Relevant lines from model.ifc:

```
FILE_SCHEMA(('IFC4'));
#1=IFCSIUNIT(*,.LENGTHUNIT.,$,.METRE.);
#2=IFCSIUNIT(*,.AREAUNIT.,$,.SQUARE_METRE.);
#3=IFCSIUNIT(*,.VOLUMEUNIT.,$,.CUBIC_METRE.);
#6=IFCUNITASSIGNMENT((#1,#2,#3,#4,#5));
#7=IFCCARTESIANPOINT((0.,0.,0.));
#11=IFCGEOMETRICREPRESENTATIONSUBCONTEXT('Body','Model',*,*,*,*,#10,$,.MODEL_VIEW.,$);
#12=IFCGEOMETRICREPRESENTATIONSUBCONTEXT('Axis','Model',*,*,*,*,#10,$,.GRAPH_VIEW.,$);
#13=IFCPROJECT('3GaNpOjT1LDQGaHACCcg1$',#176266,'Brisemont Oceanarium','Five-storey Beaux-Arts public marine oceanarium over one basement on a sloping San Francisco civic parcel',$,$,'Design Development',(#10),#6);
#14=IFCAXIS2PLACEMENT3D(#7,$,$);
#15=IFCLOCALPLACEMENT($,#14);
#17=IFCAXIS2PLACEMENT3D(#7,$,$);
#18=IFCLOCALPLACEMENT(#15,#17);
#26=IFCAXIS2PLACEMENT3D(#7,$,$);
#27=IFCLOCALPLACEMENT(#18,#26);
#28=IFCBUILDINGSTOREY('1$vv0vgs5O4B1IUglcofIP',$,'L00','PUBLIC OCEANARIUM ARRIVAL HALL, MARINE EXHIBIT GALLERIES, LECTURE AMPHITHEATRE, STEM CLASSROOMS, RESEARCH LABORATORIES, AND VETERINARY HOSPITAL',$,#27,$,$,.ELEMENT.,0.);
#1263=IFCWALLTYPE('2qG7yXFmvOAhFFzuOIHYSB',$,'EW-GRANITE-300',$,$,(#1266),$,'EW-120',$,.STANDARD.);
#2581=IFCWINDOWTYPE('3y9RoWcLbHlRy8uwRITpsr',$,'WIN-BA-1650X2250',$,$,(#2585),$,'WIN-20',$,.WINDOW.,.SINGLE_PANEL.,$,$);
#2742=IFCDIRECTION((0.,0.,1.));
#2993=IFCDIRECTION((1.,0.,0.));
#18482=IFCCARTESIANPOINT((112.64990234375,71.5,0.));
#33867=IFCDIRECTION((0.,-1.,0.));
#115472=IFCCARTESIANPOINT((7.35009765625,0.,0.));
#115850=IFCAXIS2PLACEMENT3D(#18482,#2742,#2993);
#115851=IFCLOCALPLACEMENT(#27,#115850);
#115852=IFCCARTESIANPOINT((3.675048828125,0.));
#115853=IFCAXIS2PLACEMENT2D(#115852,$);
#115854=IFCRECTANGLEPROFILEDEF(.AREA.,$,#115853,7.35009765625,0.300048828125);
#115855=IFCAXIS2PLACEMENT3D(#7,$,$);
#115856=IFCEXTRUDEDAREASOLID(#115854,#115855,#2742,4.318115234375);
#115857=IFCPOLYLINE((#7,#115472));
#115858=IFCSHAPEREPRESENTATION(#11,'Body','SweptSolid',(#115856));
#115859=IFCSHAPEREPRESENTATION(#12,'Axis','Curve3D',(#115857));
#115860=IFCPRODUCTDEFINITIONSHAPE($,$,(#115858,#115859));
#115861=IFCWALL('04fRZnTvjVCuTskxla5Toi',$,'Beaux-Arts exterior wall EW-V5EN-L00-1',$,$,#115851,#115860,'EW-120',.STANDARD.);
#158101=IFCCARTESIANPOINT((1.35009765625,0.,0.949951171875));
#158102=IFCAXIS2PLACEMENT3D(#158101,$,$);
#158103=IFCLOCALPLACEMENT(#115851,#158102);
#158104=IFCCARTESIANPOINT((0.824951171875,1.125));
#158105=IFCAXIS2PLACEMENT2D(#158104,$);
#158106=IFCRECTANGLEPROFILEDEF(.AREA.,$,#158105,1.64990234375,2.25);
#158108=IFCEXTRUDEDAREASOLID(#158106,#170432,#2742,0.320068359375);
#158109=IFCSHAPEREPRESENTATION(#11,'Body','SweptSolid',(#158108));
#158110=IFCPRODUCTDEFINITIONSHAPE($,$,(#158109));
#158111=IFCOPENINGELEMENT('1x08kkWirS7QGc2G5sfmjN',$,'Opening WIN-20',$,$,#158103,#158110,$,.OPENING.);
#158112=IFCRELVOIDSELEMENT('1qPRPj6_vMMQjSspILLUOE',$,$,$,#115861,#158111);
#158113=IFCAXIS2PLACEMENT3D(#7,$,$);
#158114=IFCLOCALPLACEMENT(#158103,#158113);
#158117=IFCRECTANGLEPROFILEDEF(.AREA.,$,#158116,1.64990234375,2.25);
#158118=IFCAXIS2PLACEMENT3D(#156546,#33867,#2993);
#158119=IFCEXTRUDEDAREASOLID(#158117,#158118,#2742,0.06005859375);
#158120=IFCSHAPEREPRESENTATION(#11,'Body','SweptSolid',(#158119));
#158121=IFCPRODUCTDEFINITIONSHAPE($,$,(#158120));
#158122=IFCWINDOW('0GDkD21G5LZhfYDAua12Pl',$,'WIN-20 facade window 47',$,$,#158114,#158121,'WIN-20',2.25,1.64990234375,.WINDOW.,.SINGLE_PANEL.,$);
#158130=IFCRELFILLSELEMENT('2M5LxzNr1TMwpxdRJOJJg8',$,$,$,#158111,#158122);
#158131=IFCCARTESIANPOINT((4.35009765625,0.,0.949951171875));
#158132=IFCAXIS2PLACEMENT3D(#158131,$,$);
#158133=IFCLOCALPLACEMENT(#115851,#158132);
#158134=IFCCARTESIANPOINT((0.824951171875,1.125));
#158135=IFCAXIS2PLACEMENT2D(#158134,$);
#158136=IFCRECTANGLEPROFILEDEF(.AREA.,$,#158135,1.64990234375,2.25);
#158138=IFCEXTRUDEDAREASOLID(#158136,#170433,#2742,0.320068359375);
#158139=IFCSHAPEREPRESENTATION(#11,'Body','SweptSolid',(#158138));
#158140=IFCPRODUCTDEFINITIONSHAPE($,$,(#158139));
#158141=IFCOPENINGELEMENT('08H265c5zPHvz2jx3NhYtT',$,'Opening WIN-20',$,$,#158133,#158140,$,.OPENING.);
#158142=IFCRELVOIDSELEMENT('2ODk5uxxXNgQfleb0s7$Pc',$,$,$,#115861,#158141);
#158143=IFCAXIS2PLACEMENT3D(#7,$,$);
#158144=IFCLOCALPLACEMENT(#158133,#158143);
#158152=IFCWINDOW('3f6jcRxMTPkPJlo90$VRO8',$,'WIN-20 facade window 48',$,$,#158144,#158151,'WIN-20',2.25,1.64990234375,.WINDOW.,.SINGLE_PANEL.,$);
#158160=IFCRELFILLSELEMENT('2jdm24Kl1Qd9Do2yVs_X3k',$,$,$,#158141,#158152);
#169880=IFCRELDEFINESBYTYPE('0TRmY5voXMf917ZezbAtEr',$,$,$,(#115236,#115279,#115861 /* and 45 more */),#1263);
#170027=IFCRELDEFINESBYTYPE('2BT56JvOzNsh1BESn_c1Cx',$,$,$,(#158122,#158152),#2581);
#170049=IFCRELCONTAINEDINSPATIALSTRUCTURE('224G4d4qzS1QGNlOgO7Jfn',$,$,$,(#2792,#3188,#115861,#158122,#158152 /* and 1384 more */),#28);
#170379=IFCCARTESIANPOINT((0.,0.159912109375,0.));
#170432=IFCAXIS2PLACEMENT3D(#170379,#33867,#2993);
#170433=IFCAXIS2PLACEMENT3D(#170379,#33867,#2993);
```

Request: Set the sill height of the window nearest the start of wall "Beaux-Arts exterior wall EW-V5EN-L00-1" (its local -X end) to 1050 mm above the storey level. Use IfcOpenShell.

```python
import numpy as np
import ifcopenshell
import ifcopenshell.api.geometry
import ifcopenshell.geom
import ifcopenshell.util.element
import ifcopenshell.util.placement
import ifcopenshell.util.shape
import ifcopenshell.util.unit

model = ifcopenshell.open("model.ifc")
unit_scale = ifcopenshell.util.unit.calculate_unit_scale(model)

window = model.by_id(158122)
opening = window.FillsVoids[0].RelatingOpeningElement
storey = ifcopenshell.util.element.get_container(window, ifc_class="IfcBuildingStorey")
level = ifcopenshell.util.placement.get_local_placement(storey.ObjectPlacement)[2, 3]

# The opening's origin need not be at the sill, so measure its lowest point.
shape = ifcopenshell.geom.create_shape(ifcopenshell.geom.settings(), opening)
bottom = ifcopenshell.util.shape.get_shape_bottom_elevation(shape, shape.geometry) / unit_scale
dz = level + 1.05 / unit_scale - bottom

shift = np.array([0.0, 0.0, dz])
# The window is placed relative to its opening, so it follows when the opening moves.
matrix = ifcopenshell.util.placement.get_local_placement(opening.ObjectPlacement)
matrix[:3, 3] += shift
ifcopenshell.api.geometry.edit_object_placement(
    model, product=opening, matrix=matrix, is_si=False, should_transform_children=True
)

print(f"moved by {dz * unit_scale:+.3f} m")

model.write("model_v2.ifc")
```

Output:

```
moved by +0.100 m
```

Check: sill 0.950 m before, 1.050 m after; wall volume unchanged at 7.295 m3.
